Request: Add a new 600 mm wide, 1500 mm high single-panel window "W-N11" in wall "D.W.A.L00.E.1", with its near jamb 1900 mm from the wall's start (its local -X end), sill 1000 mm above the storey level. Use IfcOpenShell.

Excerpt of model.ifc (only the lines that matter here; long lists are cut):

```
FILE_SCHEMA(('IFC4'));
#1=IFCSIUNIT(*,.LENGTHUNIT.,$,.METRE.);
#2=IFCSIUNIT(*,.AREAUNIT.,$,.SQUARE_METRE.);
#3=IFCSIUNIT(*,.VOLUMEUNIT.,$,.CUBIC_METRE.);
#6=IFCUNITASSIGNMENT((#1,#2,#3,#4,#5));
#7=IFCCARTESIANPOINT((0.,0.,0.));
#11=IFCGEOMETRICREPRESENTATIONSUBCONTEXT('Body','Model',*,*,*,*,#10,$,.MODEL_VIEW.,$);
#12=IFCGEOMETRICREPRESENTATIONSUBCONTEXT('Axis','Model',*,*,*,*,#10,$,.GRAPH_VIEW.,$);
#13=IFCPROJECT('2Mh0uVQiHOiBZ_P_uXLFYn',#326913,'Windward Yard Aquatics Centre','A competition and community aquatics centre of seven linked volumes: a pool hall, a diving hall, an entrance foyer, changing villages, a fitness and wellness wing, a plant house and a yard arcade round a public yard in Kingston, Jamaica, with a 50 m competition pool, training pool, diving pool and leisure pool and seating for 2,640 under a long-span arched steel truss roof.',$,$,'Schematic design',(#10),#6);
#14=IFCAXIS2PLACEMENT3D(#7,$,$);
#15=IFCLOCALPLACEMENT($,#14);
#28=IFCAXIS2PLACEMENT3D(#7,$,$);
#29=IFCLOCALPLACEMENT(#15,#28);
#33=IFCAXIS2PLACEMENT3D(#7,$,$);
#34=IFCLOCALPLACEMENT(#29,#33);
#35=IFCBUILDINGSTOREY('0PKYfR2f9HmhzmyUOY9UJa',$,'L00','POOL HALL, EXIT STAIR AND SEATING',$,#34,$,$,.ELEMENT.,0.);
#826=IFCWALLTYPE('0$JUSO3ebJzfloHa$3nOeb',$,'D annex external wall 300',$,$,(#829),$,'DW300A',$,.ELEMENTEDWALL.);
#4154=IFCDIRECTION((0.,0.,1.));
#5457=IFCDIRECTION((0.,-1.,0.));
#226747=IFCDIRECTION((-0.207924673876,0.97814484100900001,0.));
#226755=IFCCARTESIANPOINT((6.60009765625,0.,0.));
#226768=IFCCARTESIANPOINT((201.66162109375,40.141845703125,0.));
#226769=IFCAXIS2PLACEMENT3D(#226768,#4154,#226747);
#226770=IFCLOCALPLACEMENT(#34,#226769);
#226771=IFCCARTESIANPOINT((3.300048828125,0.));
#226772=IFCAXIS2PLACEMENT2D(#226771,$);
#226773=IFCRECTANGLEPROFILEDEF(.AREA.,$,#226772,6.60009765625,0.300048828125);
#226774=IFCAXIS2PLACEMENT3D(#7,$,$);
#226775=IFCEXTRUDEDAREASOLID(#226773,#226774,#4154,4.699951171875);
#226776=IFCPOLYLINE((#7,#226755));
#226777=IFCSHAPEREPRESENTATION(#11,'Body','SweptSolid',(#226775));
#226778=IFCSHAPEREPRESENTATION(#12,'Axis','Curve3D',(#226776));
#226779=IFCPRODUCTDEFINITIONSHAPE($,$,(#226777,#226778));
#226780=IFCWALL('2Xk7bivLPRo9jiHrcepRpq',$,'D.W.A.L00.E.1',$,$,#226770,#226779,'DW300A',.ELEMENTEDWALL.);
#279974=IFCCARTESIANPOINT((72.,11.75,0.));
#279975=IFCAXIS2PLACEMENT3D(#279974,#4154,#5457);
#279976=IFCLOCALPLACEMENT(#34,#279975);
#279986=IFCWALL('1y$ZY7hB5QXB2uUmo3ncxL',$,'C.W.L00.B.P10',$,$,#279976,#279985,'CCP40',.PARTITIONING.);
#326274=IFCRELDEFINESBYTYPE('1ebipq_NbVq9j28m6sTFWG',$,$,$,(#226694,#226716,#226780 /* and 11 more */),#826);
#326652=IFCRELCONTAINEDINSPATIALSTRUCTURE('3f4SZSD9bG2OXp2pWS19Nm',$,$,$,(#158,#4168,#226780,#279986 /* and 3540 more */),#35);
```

```python
import numpy as np
import ifcopenshell
import ifcopenshell.api.feature
import ifcopenshell.api.geometry
import ifcopenshell.api.root
import ifcopenshell.api.spatial
import ifcopenshell.geom
import ifcopenshell.util.element
import ifcopenshell.util.placement
import ifcopenshell.util.representation
import ifcopenshell.util.shape
import ifcopenshell.util.unit

model = ifcopenshell.open("model.ifc")
unit_scale = ifcopenshell.util.unit.calculate_unit_scale(model)
settings = ifcopenshell.geom.settings()


def volume(element):
    """Net volume in cubic metres, openings subtracted."""
    shape = ifcopenshell.geom.create_shape(settings, element)
    return ifcopenshell.util.shape.get_volume(shape.geometry)


wall = model.by_guid("2Xk7bivLPRo9jiHrcepRpq")
storey = ifcopenshell.util.element.get_container(wall, ifc_class="IfcBuildingStorey")
context = ifcopenshell.util.representation.get_context(model, "Model", "Body", "MODEL_VIEW")
before = volume(wall)

width, height, from_end, sill = 0.6, 1.5, 1.9, 1  # metres

# The wall runs along its own X axis, and the end named is its -X end.
wall_shape = ifcopenshell.geom.create_shape(settings, wall)
x, y, z = ifcopenshell.util.shape.get_vertices(wall_shape.geometry).T
start = x.min() + from_end
face, thickness = float(y.min()), float(y.max() - y.min())
wall_matrix = ifcopenshell.util.placement.get_local_placement(wall.ObjectPlacement)
level = ifcopenshell.util.placement.get_local_placement(storey.ObjectPlacement)[2, 3]


def in_wall(x, y):
    """Placement at x, y metres in the wall's axes, at sill height."""
    matrix = wall_matrix.copy()
    matrix[:, 3] = wall_matrix @ np.array([x / unit_scale, y / unit_scale, 0.0, 1.0])
    matrix[2, 3] = level + sill / unit_scale
    return matrix


# Opening: a box that overshoots both wall faces by 50 mm.
opening = ifcopenshell.api.root.create_entity(model, ifc_class="IfcOpeningElement", predefined_type="OPENING")
box = ifcopenshell.api.geometry.add_wall_representation(
    model, context=context, length=width, height=height, thickness=thickness + 0.1
)
ifcopenshell.api.geometry.assign_representation(model, product=opening, representation=box)
ifcopenshell.api.geometry.edit_object_placement(model, product=opening, matrix=in_wall(start, face - 0.05), is_si=False)
ifcopenshell.api.feature.add_feature(model, feature=opening, element=wall)

window = ifcopenshell.api.root.create_entity(model, ifc_class="IfcWindow", name="W-N11", predefined_type="WINDOW")
window.OverallWidth, window.OverallHeight = width / unit_scale, height / unit_scale
window.PartitioningType = "SINGLE_PANEL"
body = ifcopenshell.api.geometry.add_window_representation(
    model,
    context=context,
    overall_width=window.OverallWidth,
    overall_height=window.OverallHeight,
    partition_type="SINGLE_PANEL",
)
ifcopenshell.api.geometry.assign_representation(model, product=window, representation=body)
ifcopenshell.api.spatial.assign_container(model, products=[window], relating_structure=storey)
ifcopenshell.api.feature.add_filling(model, opening=opening, element=window)

# Centre the window in the wall's thickness.
ifcopenshell.api.geometry.edit_object_placement(model, product=window, matrix=in_wall(start, face), is_si=False)
window_shape = ifcopenshell.geom.create_shape(settings, window)
depth = ifcopenshell.util.shape.get_vertices(window_shape.geometry)[:, 1]
offset = face + thickness / 2 - (depth.min() + depth.max()) / 2
ifcopenshell.api.geometry.edit_object_placement(model, product=window, matrix=in_wall(start, offset), is_si=False)

after = volume(wall)

print(f"wall volume {before:.3f} -> {after:.3f} m3")

model.write("model_updated.ifc")
```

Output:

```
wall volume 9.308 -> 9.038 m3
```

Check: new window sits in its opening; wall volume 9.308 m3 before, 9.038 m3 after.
